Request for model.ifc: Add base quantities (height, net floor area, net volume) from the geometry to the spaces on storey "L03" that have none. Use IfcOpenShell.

First a look at what the model holds.

```python
import ifcopenshell
import ifcopenshell.util.element
import ifcopenshell.util.unit

model = ifcopenshell.open("model.ifc")
print(model.schema)
for unit_type in ("LENGTHUNIT", "AREAUNIT", "VOLUMEUNIT"):
    print(unit_type, ifcopenshell.util.unit.calculate_unit_scale(model, unit_type))
storey = next(s for s in model.by_type("IfcBuildingStorey") if s.Name == "L03")
spaces = [e for e in ifcopenshell.util.element.get_decomposition(storey) if e.is_a("IfcSpace")]
for e in sorted(spaces, key=lambda e: e.id()):
    print(e.id(), e.is_a(), e.Name, list(ifcopenshell.util.element.get_psets(e, qtos_only=True)), sep=" | ")
```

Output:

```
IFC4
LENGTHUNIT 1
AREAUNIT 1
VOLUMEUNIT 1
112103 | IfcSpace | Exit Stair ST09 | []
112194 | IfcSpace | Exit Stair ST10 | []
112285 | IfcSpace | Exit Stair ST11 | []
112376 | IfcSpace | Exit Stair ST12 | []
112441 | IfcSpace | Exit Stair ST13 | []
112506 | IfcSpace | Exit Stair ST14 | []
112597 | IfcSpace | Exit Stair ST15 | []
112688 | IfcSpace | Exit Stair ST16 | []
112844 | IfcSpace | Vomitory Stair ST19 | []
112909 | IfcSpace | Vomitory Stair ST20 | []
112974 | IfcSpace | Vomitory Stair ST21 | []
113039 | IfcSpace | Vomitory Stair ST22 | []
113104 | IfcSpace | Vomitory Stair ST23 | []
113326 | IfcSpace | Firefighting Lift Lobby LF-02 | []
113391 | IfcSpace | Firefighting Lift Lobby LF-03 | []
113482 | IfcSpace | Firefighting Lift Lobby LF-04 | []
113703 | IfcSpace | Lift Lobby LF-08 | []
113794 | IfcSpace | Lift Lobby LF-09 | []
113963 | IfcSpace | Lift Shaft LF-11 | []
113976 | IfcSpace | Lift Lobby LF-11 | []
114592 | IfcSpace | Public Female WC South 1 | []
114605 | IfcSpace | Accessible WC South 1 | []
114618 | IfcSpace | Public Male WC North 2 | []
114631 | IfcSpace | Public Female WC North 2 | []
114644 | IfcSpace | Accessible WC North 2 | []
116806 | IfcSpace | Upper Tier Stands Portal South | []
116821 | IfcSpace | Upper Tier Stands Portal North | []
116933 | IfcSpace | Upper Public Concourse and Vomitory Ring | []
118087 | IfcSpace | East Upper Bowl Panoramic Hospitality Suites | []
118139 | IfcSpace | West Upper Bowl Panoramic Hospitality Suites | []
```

```python
import ifcopenshell
import ifcopenshell.api.pset
import ifcopenshell.geom
import ifcopenshell.util.element
import ifcopenshell.util.shape
import ifcopenshell.util.unit

model = ifcopenshell.open("model.ifc")
unit_scale = ifcopenshell.util.unit.calculate_unit_scale(model)
area_scale = ifcopenshell.util.unit.calculate_unit_scale(model, "AREAUNIT")
volume_scale = ifcopenshell.util.unit.calculate_unit_scale(model, "VOLUMEUNIT")
settings = ifcopenshell.geom.settings()

storey = next(s for s in model.by_type("IfcBuildingStorey") if s.Name == "L03")
spaces = [e for e in ifcopenshell.util.element.get_decomposition(storey) if e.is_a("IfcSpace")]

for e in sorted(spaces, key=lambda e: e.id()):
    if ifcopenshell.util.element.get_psets(e, qtos_only=True, should_inherit=False):
        continue
    # Geometry comes back in metres, in the element's own axes.
    shape = ifcopenshell.geom.create_shape(settings, e)
    values = {
        "Height": ifcopenshell.util.shape.get_z(shape.geometry) / unit_scale,
        "NetFloorArea": ifcopenshell.util.shape.get_footprint_area(shape.geometry) / area_scale,
        "NetVolume": ifcopenshell.util.shape.get_volume(shape.geometry) / volume_scale,
    }
    qto = ifcopenshell.api.pset.add_qto(model, product=e, name="Qto_SpaceBaseQuantities")
    ifcopenshell.api.pset.edit_qto(model, qto=qto, properties=values)
    print(e.id(), {k: round(v, 3) for k, v in values.items()})

model.write("model_v2.ifc")
```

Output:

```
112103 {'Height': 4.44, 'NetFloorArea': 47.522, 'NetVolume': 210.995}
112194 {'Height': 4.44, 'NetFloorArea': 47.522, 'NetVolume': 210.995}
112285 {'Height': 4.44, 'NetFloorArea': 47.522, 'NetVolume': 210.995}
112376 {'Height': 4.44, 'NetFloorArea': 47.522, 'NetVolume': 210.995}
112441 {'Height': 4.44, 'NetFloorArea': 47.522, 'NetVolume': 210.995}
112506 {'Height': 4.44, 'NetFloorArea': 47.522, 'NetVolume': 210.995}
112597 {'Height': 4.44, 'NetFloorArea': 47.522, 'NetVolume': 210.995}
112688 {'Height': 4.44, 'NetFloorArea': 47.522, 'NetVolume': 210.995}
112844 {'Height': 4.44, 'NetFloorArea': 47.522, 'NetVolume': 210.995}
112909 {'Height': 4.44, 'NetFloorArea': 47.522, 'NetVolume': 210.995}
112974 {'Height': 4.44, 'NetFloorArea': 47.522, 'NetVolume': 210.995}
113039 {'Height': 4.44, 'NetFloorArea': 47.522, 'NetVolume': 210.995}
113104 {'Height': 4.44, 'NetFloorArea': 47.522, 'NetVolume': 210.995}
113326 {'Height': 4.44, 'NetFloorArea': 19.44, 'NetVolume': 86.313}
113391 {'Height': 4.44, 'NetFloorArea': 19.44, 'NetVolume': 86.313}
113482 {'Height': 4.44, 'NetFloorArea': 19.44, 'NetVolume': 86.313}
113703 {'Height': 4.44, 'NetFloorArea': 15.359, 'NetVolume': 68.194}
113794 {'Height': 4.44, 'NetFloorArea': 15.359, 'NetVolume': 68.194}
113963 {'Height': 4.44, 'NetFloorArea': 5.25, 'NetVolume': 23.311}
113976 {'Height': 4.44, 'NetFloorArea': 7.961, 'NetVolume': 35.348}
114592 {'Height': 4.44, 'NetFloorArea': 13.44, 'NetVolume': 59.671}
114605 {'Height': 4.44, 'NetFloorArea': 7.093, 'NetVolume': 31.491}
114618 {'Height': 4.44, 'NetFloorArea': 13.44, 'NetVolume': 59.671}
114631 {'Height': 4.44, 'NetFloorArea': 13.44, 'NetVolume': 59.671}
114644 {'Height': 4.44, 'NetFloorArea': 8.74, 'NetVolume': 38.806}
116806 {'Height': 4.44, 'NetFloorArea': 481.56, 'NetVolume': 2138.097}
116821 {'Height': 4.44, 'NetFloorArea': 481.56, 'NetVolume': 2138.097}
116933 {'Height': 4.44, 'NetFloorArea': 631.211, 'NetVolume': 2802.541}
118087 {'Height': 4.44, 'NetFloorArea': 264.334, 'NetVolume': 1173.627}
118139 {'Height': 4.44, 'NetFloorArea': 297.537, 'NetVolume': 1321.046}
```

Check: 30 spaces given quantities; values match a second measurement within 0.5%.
